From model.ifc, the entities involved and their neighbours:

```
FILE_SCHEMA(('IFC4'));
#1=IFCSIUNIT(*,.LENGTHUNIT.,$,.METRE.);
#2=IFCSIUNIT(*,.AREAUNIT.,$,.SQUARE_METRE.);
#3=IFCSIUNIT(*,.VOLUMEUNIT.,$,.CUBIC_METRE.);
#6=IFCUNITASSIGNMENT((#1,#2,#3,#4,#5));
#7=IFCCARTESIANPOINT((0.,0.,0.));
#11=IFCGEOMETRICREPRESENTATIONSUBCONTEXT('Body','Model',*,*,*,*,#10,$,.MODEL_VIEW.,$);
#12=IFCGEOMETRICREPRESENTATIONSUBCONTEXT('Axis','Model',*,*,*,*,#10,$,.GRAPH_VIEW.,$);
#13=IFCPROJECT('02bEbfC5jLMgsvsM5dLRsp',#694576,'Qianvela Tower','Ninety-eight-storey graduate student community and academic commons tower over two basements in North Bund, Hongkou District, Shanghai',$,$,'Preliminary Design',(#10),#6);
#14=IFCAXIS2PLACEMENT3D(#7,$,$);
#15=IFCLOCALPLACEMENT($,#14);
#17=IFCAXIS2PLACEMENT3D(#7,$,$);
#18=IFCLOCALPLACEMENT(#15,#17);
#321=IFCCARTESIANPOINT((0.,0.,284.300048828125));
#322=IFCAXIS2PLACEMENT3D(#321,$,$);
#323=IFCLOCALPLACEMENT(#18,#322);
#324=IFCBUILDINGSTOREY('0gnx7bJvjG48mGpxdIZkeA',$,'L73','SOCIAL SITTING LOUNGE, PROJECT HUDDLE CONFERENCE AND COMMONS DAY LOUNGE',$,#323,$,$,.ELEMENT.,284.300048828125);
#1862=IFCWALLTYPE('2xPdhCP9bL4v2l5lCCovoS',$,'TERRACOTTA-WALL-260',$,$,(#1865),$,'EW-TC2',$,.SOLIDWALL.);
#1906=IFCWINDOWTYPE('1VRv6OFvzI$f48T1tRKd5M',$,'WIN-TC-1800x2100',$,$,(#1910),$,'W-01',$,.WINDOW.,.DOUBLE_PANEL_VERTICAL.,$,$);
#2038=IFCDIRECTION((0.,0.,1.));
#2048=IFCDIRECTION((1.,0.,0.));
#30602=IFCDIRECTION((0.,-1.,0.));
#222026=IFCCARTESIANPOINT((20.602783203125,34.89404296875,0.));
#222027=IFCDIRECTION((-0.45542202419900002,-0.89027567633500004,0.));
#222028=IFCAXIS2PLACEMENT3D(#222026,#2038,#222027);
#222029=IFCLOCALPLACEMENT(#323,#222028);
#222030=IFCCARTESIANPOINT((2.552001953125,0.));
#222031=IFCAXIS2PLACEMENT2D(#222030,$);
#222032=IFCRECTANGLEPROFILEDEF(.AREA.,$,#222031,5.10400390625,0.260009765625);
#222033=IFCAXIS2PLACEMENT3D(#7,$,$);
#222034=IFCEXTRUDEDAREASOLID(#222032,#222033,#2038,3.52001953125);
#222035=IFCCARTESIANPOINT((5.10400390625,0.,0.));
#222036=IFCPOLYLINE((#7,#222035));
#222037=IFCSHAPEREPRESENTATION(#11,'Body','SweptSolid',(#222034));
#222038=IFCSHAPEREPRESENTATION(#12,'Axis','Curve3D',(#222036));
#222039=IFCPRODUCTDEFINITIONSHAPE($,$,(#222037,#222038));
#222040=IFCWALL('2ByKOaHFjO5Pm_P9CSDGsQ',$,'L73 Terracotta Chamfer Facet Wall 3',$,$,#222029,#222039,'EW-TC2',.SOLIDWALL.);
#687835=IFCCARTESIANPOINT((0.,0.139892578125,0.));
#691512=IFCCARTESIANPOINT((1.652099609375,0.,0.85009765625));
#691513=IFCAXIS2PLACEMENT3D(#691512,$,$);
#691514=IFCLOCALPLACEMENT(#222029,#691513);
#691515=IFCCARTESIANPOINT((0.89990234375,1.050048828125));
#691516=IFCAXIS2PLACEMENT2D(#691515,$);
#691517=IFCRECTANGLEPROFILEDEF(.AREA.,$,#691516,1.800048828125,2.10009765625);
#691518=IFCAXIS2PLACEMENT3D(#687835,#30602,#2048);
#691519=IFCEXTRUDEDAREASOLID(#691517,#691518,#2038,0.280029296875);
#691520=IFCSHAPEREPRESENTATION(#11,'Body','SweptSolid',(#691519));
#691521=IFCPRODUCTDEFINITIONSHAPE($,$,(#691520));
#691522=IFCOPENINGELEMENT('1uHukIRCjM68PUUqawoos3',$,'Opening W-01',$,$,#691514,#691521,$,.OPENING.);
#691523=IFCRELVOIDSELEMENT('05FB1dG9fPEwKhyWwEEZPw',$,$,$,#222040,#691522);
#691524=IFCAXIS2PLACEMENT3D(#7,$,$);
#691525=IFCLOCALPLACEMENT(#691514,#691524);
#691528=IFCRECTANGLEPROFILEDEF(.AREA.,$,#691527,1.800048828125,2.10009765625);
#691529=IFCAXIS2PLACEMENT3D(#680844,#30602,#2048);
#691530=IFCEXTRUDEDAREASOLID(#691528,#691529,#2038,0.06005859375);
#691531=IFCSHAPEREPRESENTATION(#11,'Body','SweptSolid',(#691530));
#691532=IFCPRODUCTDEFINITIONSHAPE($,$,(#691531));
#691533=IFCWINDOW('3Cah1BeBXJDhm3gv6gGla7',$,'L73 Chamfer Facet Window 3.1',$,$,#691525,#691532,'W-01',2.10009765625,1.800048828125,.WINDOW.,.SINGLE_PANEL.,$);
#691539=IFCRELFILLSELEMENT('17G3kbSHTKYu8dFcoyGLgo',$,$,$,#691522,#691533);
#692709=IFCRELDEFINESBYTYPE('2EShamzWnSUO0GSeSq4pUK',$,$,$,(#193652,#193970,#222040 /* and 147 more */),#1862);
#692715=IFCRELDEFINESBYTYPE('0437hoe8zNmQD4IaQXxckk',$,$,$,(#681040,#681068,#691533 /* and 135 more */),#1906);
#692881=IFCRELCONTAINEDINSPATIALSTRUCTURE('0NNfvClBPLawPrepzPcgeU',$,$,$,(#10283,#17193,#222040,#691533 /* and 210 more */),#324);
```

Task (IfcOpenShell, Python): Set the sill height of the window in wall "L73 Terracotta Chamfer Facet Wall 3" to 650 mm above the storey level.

```python
import numpy as np
import ifcopenshell
import ifcopenshell.api.geometry
import ifcopenshell.geom
import ifcopenshell.util.element
import ifcopenshell.util.placement
import ifcopenshell.util.shape
import ifcopenshell.util.unit

model = ifcopenshell.open("model.ifc")
unit_scale = ifcopenshell.util.unit.calculate_unit_scale(model)

window = model.by_guid("3Cah1BeBXJDhm3gv6gGla7")
opening = window.FillsVoids[0].RelatingOpeningElement
storey = ifcopenshell.util.element.get_container(window, ifc_class="IfcBuildingStorey")
level = ifcopenshell.util.placement.get_local_placement(storey.ObjectPlacement)[2, 3]

# The opening's origin need not be at the sill, so measure its lowest point.
shape = ifcopenshell.geom.create_shape(ifcopenshell.geom.settings(), opening)
bottom = ifcopenshell.util.shape.get_shape_bottom_elevation(shape, shape.geometry) / unit_scale
dz = level + 0.65 - bottom

shift = np.array([0.0, 0.0, dz])
# The window is placed relative to its opening, so it follows when the opening moves.
matrix = ifcopenshell.util.placement.get_local_placement(opening.ObjectPlacement)
matrix[:3, 3] += shift
ifcopenshell.api.geometry.edit_object_placement(
    model, product=opening, matrix=matrix, is_si=False, should_transform_children=True
)

print(f"moved by {dz * unit_scale:+.3f} m")

model.write("model-out.ifc")
```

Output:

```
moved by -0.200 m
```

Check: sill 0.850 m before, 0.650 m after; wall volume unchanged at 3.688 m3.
